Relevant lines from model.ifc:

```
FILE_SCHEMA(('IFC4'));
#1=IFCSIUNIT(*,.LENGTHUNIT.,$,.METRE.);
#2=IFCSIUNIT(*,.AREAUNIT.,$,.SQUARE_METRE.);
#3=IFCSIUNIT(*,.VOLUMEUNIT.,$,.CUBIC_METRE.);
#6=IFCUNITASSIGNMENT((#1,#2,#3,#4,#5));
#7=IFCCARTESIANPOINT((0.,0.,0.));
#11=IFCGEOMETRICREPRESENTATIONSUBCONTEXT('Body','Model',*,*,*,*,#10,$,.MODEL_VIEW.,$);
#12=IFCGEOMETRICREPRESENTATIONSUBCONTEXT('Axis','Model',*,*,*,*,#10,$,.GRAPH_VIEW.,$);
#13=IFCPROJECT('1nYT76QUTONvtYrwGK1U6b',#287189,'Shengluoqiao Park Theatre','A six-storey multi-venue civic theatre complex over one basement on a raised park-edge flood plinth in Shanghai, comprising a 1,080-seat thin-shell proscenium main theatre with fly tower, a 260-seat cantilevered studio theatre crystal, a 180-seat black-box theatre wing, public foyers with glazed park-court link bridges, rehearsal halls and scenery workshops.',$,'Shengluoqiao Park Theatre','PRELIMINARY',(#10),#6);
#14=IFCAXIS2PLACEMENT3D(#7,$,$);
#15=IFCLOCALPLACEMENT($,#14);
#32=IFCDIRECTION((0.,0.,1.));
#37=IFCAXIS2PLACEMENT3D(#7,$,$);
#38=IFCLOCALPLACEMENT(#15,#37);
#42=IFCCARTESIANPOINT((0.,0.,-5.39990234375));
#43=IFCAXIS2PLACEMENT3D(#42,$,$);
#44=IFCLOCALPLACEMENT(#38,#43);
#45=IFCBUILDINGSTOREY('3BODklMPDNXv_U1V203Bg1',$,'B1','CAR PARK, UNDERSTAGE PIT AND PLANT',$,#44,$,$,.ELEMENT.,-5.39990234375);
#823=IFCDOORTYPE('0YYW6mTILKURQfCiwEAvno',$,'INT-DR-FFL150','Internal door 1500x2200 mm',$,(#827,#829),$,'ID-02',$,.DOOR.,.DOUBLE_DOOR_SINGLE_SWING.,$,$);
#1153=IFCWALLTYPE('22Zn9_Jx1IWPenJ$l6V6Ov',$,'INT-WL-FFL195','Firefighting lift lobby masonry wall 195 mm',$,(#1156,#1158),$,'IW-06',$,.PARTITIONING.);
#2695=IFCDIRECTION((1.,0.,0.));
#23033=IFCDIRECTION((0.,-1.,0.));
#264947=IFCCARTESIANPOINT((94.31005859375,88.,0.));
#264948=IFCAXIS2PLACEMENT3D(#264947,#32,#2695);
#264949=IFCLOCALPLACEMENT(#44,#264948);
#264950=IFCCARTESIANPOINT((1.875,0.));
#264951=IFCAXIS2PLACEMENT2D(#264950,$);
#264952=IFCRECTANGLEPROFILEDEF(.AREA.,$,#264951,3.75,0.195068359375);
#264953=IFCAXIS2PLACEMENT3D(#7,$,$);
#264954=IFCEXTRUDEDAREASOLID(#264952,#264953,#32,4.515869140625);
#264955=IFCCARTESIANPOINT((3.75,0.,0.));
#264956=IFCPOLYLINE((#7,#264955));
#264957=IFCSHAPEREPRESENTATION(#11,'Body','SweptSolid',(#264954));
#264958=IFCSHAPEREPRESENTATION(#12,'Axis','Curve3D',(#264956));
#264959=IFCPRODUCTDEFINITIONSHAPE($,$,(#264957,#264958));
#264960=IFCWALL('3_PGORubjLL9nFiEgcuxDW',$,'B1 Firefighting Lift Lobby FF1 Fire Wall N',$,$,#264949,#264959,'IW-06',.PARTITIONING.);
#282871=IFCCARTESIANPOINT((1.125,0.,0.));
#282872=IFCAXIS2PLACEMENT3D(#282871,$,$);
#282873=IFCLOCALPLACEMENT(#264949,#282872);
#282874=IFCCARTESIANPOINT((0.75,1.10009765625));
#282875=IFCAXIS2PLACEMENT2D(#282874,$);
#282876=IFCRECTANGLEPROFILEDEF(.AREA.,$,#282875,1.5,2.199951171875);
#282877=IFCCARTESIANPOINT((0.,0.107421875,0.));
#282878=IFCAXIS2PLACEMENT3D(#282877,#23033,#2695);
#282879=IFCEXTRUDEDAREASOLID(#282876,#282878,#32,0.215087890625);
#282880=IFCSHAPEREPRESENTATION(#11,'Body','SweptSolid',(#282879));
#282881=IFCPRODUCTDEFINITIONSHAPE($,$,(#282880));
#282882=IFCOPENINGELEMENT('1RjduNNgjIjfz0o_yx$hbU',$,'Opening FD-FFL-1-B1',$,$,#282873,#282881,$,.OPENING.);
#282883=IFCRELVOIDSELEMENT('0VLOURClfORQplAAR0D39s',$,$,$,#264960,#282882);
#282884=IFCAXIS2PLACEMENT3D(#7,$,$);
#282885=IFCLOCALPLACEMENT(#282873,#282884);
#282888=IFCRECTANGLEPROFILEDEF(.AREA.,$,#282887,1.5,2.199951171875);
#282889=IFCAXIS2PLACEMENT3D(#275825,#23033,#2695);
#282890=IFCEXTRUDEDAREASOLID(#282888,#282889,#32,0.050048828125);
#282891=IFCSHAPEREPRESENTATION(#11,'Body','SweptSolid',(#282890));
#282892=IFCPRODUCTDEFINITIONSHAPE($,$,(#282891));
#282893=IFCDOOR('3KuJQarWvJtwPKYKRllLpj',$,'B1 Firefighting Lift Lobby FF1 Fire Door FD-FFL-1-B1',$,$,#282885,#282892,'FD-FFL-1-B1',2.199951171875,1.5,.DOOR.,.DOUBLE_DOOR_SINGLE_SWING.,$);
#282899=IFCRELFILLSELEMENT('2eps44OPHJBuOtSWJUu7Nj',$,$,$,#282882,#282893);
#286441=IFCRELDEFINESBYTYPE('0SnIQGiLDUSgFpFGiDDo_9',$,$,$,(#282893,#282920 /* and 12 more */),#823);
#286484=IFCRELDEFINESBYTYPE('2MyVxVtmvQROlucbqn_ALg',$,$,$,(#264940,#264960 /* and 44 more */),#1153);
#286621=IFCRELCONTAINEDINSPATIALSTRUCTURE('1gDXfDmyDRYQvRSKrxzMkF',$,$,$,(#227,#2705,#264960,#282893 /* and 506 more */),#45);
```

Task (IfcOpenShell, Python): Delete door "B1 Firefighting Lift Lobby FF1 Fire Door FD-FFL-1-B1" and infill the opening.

```python
import ifcopenshell
import ifcopenshell.api.feature
import ifcopenshell.api.root
import ifcopenshell.geom
import ifcopenshell.util.shape

model = ifcopenshell.open("model.ifc")
settings = ifcopenshell.geom.settings()


def volume(element):
    """Net volume in cubic metres, openings subtracted."""
    shape = ifcopenshell.geom.create_shape(settings, element)
    return ifcopenshell.util.shape.get_volume(shape.geometry)


door = model.by_id(282893)
opening = door.FillsVoids[0].RelatingOpeningElement
wall = opening.VoidsElements[0].RelatingBuildingElement
before = volume(wall)

ifcopenshell.api.root.remove_product(model, product=door)
ifcopenshell.api.feature.remove_feature(model, feature=opening)

after = volume(wall)

print(f"wall volume {before:.3f} -> {after:.3f} m3")

model.write("model_edited.ifc")
```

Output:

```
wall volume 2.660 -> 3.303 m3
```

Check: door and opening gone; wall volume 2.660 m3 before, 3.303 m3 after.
